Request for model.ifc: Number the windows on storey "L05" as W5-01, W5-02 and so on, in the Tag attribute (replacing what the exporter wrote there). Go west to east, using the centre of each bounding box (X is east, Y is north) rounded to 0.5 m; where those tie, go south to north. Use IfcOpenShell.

First a look at what the model holds.

```python
import ifcopenshell
import ifcopenshell.util.element
import ifcopenshell.util.placement

model = ifcopenshell.open("model.ifc")
print(model.schema)
storey = next(s for s in model.by_type("IfcBuildingStorey") if s.Name == "L05")
windows = [e for e in ifcopenshell.util.element.get_decomposition(storey) if e.is_a("IfcWindow")]
for e in sorted(windows, key=lambda e: e.id()):
    origin = ifcopenshell.util.placement.get_local_placement(e.ObjectPlacement)[:3, 3]
    print(e.id(), e.Tag, e.Name, origin.round(2) + 0.0, sep=" | ")
```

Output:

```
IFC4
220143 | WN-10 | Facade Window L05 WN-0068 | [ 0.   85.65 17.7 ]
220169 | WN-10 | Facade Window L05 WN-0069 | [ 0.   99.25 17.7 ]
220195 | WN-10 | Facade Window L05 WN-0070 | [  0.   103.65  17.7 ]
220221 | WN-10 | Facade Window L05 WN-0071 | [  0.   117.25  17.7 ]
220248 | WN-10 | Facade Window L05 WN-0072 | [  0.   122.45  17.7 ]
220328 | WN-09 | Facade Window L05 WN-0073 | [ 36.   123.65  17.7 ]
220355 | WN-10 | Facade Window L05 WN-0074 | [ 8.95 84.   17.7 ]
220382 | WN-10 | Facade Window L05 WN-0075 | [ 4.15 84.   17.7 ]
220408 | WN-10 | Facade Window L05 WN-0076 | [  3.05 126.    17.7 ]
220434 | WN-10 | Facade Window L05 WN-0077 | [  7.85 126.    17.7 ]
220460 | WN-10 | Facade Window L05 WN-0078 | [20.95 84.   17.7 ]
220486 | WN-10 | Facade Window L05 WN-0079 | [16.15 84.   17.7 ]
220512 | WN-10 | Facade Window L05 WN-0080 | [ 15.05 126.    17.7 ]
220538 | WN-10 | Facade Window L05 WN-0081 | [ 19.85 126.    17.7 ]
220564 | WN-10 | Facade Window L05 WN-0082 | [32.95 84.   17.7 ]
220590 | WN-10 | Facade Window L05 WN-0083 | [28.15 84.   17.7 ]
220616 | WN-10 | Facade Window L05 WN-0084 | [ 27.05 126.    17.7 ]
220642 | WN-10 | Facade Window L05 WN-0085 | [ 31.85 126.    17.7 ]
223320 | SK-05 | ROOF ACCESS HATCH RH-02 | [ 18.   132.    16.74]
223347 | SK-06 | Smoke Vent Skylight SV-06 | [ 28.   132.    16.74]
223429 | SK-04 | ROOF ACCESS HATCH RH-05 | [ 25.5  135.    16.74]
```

```python
import ifcopenshell
import ifcopenshell.geom
import ifcopenshell.util.element
import ifcopenshell.util.shape

model = ifcopenshell.open("model.ifc")
settings = ifcopenshell.geom.settings()
settings.set("use-world-coords", True)


def centre(element):
    shape = ifcopenshell.geom.create_shape(settings, element)
    return ifcopenshell.util.shape.get_bbox_centroid(shape.geometry)


storey = next(s for s in model.by_type("IfcBuildingStorey") if s.Name == "L05")
windows = [e for e in ifcopenshell.util.element.get_decomposition(storey) if e.is_a("IfcWindow")]

# Insertion points can sit at a corner or the storey origin, so sort by the geometry (in metres).
centres = {e: centre(e) for e in windows}
windows.sort(key=lambda e: (round(centres[e][0] / 0.5), centres[e][1]))

for i, e in enumerate(windows, start=1):
    number = f"W5-{i:02d}"
    e.Tag = number
    print(e.id(), number)

model.write("model_rev.ifc")
```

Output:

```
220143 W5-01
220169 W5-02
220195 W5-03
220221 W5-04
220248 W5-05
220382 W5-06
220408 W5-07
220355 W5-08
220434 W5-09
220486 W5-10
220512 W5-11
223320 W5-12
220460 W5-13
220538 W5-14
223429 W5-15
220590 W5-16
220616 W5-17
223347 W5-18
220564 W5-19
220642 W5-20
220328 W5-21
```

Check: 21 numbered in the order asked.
